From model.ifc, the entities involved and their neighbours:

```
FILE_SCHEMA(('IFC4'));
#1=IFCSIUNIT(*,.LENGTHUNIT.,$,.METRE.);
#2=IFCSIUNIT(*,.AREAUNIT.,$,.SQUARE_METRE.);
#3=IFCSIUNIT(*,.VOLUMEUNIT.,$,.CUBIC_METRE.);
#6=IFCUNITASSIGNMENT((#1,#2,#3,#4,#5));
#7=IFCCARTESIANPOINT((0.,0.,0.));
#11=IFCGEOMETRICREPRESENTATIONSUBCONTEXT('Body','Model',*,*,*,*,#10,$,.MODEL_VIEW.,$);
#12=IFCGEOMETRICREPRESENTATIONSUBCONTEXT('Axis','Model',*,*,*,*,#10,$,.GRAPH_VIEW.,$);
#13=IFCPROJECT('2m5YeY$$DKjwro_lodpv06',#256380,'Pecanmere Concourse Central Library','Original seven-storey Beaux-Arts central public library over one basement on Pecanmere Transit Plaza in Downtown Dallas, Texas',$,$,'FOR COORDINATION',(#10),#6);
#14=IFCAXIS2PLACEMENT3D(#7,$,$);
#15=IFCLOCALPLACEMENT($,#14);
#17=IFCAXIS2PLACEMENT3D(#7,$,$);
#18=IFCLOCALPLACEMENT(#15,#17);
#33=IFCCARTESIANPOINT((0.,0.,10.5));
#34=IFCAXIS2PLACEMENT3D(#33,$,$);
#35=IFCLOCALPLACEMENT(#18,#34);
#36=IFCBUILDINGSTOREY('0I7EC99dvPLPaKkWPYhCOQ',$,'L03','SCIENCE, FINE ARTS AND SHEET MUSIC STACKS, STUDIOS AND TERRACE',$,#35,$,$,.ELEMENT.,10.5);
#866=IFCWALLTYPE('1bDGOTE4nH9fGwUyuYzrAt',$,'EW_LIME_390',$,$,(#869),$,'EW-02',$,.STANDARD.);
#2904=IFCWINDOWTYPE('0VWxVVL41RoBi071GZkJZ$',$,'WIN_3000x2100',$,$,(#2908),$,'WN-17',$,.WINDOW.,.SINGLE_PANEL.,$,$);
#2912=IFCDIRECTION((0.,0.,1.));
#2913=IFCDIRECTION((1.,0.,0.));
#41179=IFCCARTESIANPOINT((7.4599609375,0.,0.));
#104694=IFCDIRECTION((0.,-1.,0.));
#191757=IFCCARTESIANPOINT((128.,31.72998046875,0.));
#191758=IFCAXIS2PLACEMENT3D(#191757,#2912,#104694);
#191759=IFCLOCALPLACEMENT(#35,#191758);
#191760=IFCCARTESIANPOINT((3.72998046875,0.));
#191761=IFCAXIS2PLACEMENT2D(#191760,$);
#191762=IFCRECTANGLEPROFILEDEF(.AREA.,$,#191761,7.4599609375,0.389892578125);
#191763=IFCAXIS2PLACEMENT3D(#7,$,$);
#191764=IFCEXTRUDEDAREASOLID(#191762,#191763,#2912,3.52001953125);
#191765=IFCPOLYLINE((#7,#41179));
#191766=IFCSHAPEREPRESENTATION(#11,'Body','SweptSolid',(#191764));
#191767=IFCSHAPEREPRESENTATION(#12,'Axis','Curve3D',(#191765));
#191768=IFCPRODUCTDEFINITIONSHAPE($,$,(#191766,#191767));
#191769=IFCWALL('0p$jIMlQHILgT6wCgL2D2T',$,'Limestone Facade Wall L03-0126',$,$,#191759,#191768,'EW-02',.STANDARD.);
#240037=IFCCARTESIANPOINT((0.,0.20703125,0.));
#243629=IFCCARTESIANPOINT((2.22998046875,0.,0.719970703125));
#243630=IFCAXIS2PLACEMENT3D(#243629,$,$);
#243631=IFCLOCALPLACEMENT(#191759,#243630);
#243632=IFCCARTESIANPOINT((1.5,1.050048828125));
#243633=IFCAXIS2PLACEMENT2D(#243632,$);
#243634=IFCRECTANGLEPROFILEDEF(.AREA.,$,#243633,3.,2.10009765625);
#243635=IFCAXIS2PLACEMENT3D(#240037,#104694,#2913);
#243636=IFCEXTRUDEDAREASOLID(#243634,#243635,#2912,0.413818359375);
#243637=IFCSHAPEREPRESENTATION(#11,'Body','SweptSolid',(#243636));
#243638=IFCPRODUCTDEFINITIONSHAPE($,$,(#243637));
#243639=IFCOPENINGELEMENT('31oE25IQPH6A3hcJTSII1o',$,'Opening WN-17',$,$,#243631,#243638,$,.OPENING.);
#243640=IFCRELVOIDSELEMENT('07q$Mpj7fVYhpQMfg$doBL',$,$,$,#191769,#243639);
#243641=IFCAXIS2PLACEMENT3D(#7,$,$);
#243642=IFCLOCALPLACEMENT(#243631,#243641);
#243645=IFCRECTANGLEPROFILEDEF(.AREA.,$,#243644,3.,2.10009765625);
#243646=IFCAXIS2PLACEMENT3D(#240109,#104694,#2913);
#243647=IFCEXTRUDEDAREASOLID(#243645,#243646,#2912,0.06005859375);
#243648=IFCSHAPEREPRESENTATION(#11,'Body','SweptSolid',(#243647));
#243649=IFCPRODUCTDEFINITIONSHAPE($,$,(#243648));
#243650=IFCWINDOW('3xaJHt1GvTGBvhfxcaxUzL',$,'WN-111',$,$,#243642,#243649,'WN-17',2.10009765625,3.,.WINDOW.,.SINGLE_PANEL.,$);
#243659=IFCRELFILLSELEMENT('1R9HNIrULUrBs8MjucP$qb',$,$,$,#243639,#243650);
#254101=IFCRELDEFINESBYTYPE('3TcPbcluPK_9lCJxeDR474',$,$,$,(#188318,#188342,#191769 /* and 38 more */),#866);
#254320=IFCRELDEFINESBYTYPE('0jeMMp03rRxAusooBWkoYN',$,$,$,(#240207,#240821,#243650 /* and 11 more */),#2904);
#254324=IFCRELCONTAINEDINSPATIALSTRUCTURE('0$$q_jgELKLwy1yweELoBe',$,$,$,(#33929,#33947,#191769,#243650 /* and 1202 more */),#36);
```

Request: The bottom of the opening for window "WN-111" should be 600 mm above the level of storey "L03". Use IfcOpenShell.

```python
import numpy as np
import ifcopenshell
import ifcopenshell.api.geometry
import ifcopenshell.geom
import ifcopenshell.util.element
import ifcopenshell.util.placement
import ifcopenshell.util.shape
import ifcopenshell.util.unit

model = ifcopenshell.open("model.ifc")
unit_scale = ifcopenshell.util.unit.calculate_unit_scale(model)

window = model.by_guid("3xaJHt1GvTGBvhfxcaxUzL")
opening = window.FillsVoids[0].RelatingOpeningElement
storey = ifcopenshell.util.element.get_container(window, ifc_class="IfcBuildingStorey")
level = ifcopenshell.util.placement.get_local_placement(storey.ObjectPlacement)[2, 3]

# The opening's origin need not be at the sill, so measure its lowest point.
shape = ifcopenshell.geom.create_shape(ifcopenshell.geom.settings(), opening)
bottom = ifcopenshell.util.shape.get_shape_bottom_elevation(shape, shape.geometry) / unit_scale
dz = level + 0.6 / unit_scale - bottom

shift = np.array([0.0, 0.0, dz])
# The window is placed relative to its opening, so it follows when the opening moves.
matrix = ifcopenshell.util.placement.get_local_placement(opening.ObjectPlacement)
matrix[:3, 3] += shift
ifcopenshell.api.geometry.edit_object_placement(
    model, product=opening, matrix=matrix, is_si=False, should_transform_children=True
)

print(f"moved by {dz * unit_scale:+.3f} m")

model.write("model_edited.ifc")
```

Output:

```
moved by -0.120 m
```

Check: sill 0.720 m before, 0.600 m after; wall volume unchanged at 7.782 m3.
